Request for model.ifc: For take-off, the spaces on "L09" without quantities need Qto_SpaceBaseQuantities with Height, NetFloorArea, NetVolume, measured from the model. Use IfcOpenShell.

First a look at what the model holds.

```python
import ifcopenshell
import ifcopenshell.util.element
import ifcopenshell.util.unit

model = ifcopenshell.open("model.ifc")
print(model.schema)
for unit_type in ("LENGTHUNIT", "AREAUNIT", "VOLUMEUNIT"):
    print(unit_type, ifcopenshell.util.unit.calculate_unit_scale(model, unit_type))
storey = next(s for s in model.by_type("IfcBuildingStorey") if s.Name == "L09")
spaces = [e for e in ifcopenshell.util.element.get_decomposition(storey) if e.is_a("IfcSpace")]
for e in sorted(spaces, key=lambda e: e.id()):
    print(e.id(), e.is_a(), e.Name, list(ifcopenshell.util.element.get_psets(e, qtos_only=True)), sep=" | ")
```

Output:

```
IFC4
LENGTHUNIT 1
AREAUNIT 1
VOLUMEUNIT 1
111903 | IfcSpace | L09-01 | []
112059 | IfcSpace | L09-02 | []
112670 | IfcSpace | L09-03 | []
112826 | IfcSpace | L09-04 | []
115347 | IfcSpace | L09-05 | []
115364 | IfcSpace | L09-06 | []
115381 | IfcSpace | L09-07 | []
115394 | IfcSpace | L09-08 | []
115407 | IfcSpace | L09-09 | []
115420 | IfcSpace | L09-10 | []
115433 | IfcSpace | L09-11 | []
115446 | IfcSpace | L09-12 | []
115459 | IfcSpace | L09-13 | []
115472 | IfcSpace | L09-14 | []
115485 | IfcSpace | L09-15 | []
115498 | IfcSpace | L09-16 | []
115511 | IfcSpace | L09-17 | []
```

```python
import ifcopenshell
import ifcopenshell.api.pset
import ifcopenshell.geom
import ifcopenshell.util.element
import ifcopenshell.util.shape
import ifcopenshell.util.unit

model = ifcopenshell.open("model.ifc")
unit_scale = ifcopenshell.util.unit.calculate_unit_scale(model)
area_scale = ifcopenshell.util.unit.calculate_unit_scale(model, "AREAUNIT")
volume_scale = ifcopenshell.util.unit.calculate_unit_scale(model, "VOLUMEUNIT")
settings = ifcopenshell.geom.settings()

storey = next(s for s in model.by_type("IfcBuildingStorey") if s.Name == "L09")
spaces = [e for e in ifcopenshell.util.element.get_decomposition(storey) if e.is_a("IfcSpace")]

for e in sorted(spaces, key=lambda e: e.id()):
    if ifcopenshell.util.element.get_psets(e, qtos_only=True, should_inherit=False):
        continue
    # Geometry comes back in metres, in the element's own axes.
    shape = ifcopenshell.geom.create_shape(settings, e)
    values = {
        "Height": ifcopenshell.util.shape.get_z(shape.geometry) / unit_scale,
        "NetFloorArea": ifcopenshell.util.shape.get_footprint_area(shape.geometry) / area_scale,
        "NetVolume": ifcopenshell.util.shape.get_volume(shape.geometry) / volume_scale,
    }
    qto = ifcopenshell.api.pset.add_qto(model, product=e, name="Qto_SpaceBaseQuantities")
    ifcopenshell.api.pset.edit_qto(model, qto=qto, properties=values)
    print(e.id(), {k: round(v, 3) for k, v in values.items()})

model.write("model_edited.ifc")
```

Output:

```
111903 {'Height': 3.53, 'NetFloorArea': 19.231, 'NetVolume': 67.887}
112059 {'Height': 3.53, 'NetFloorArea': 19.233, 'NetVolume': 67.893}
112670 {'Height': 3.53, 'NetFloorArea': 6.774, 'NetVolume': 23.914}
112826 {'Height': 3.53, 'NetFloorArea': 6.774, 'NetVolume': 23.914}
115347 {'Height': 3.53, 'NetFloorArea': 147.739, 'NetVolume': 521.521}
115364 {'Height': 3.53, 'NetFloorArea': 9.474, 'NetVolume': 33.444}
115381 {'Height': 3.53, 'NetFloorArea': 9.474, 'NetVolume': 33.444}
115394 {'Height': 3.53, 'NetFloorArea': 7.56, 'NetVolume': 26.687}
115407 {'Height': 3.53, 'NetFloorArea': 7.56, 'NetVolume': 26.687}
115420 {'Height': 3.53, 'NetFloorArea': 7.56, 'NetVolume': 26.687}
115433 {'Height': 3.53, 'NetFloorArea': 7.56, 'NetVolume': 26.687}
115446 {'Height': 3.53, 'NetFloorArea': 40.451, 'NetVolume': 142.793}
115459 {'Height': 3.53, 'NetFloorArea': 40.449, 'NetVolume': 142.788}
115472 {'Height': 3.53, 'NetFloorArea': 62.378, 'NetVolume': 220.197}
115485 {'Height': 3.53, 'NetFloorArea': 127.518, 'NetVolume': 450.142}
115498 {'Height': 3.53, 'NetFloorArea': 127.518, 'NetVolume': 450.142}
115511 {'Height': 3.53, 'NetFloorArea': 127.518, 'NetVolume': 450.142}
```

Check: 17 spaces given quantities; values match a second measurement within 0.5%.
